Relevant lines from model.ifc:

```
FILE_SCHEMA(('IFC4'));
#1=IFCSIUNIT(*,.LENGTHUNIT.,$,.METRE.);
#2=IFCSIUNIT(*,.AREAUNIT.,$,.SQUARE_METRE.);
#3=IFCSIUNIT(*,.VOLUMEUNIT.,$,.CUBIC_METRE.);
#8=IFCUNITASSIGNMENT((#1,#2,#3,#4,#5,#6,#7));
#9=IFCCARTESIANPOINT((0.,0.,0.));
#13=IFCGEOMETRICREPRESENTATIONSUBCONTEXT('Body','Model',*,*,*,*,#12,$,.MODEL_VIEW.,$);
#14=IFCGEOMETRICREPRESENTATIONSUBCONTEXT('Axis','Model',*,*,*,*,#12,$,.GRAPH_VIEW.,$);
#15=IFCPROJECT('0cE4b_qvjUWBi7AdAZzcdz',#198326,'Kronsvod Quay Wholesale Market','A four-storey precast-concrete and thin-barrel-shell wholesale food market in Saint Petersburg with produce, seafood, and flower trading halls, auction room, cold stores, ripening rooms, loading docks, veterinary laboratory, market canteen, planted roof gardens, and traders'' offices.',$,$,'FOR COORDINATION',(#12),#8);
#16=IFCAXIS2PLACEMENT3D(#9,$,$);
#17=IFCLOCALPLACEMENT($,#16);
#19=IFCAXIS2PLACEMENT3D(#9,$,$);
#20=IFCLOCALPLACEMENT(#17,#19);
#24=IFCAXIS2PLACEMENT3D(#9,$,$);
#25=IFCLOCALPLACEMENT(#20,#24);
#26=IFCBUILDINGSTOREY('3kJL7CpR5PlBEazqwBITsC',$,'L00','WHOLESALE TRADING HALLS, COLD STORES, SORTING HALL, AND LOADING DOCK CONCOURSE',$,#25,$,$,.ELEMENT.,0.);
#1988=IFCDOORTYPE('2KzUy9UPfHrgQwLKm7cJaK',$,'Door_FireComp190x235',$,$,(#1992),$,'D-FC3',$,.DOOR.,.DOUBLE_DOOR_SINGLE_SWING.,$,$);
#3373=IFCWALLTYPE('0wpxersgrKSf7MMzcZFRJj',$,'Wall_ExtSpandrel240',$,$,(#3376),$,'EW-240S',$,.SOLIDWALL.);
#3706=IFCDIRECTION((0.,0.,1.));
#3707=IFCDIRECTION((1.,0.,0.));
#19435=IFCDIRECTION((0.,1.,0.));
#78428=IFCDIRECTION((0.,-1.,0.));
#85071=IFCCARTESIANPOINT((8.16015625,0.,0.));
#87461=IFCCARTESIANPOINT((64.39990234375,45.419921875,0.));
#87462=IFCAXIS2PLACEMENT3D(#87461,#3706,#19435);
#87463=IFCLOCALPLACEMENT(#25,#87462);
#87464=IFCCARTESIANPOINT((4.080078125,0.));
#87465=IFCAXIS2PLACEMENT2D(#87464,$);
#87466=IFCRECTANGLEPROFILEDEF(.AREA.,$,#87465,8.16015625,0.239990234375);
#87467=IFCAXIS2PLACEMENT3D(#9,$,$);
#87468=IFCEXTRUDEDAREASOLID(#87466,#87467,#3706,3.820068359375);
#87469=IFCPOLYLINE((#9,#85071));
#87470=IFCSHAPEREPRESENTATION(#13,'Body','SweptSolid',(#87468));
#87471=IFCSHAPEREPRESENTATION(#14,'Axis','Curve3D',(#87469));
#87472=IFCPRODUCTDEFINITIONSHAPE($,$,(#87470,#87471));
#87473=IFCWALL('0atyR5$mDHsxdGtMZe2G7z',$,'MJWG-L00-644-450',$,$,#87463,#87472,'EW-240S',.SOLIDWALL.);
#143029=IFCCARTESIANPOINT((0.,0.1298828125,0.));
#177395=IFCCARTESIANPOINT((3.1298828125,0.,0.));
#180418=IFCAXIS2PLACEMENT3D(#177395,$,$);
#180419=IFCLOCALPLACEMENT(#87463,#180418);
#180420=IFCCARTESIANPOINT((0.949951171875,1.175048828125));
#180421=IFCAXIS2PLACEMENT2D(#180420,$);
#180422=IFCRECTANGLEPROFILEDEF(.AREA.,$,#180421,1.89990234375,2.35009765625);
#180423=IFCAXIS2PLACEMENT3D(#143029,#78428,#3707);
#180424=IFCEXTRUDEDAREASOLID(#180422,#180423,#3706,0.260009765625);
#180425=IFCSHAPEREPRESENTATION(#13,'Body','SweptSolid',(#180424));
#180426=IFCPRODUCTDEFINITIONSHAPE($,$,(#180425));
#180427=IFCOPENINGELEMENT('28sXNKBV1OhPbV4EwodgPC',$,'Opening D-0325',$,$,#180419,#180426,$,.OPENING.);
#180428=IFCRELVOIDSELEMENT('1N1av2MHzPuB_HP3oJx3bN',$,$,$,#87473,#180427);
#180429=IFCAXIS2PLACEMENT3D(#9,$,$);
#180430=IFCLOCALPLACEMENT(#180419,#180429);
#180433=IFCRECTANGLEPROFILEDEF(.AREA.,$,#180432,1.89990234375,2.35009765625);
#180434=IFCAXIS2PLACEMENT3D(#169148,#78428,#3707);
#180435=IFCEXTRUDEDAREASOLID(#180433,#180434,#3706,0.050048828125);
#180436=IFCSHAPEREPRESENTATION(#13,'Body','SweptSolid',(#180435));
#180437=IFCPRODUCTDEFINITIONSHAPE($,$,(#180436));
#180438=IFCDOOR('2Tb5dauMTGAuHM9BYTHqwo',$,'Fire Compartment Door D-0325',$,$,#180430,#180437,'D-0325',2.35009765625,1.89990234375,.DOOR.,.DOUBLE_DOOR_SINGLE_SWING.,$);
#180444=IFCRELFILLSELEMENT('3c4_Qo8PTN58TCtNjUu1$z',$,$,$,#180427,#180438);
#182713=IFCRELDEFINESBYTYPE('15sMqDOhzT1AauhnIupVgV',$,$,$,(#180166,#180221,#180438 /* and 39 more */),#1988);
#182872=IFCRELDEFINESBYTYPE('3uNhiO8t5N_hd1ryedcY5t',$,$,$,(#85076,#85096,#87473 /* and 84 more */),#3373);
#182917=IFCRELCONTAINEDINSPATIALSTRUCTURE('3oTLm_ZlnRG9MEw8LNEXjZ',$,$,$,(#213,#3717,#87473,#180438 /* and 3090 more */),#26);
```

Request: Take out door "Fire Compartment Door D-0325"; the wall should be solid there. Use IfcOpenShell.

```python
import ifcopenshell
import ifcopenshell.api.feature
import ifcopenshell.api.root
import ifcopenshell.geom
import ifcopenshell.util.shape

model = ifcopenshell.open("model.ifc")
settings = ifcopenshell.geom.settings()


def volume(element):
    """Net volume in cubic metres, openings subtracted."""
    shape = ifcopenshell.geom.create_shape(settings, element)
    return ifcopenshell.util.shape.get_volume(shape.geometry)


door = model.by_guid("2Tb5dauMTGAuHM9BYTHqwo")
opening = door.FillsVoids[0].RelatingOpeningElement
wall = opening.VoidsElements[0].RelatingBuildingElement
before = volume(wall)

ifcopenshell.api.root.remove_product(model, product=door)
ifcopenshell.api.feature.remove_feature(model, feature=opening)

after = volume(wall)

print(f"wall volume {before:.3f} -> {after:.3f} m3")

model.write("model_rev.ifc")
```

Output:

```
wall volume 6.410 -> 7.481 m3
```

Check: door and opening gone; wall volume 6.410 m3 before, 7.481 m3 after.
